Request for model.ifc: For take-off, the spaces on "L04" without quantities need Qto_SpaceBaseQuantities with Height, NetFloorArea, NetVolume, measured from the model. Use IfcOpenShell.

First a look at what the model holds.

```python
import ifcopenshell
import ifcopenshell.util.element
import ifcopenshell.util.unit

model = ifcopenshell.open("model.ifc")
print(model.schema)
for unit_type in ("LENGTHUNIT", "AREAUNIT", "VOLUMEUNIT"):
    print(unit_type, ifcopenshell.util.unit.calculate_unit_scale(model, unit_type))
storey = next(s for s in model.by_type("IfcBuildingStorey") if s.Name == "L04")
spaces = [e for e in ifcopenshell.util.element.get_decomposition(storey) if e.is_a("IfcSpace")]
for e in sorted(spaces, key=lambda e: e.id()):
    print(e.id(), e.is_a(), e.Name, list(ifcopenshell.util.element.get_psets(e, qtos_only=True)), sep=" | ")
```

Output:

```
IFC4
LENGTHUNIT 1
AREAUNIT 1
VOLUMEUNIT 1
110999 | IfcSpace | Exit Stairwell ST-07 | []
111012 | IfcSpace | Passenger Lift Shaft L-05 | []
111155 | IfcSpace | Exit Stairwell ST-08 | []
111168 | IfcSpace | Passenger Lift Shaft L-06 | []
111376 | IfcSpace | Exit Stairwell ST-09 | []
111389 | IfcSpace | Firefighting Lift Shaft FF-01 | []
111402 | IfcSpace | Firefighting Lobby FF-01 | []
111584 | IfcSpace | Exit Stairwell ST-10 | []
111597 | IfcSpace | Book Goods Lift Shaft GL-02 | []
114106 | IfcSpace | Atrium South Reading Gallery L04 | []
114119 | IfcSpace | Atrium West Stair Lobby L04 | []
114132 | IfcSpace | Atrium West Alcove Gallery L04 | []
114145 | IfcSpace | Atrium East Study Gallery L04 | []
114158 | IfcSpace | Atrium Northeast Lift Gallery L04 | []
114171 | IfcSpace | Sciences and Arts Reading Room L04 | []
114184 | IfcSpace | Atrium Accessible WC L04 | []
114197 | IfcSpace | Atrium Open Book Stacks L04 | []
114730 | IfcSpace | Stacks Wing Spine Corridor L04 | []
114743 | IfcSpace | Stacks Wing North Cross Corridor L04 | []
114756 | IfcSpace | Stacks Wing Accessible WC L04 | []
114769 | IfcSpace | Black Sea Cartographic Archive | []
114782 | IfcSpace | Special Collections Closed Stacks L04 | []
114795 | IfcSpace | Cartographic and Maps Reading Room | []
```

```python
import ifcopenshell
import ifcopenshell.api.pset
import ifcopenshell.geom
import ifcopenshell.util.element
import ifcopenshell.util.shape
import ifcopenshell.util.unit

model = ifcopenshell.open("model.ifc")
unit_scale = ifcopenshell.util.unit.calculate_unit_scale(model)
area_scale = ifcopenshell.util.unit.calculate_unit_scale(model, "AREAUNIT")
volume_scale = ifcopenshell.util.unit.calculate_unit_scale(model, "VOLUMEUNIT")
settings = ifcopenshell.geom.settings()

storey = next(s for s in model.by_type("IfcBuildingStorey") if s.Name == "L04")
spaces = [e for e in ifcopenshell.util.element.get_decomposition(storey) if e.is_a("IfcSpace")]

for e in sorted(spaces, key=lambda e: e.id()):
    if ifcopenshell.util.element.get_psets(e, qtos_only=True, should_inherit=False):
        continue
    # Geometry comes back in metres, in the element's own axes.
    shape = ifcopenshell.geom.create_shape(settings, e)
    values = {
        "Height": ifcopenshell.util.shape.get_z(shape.geometry) / unit_scale,
        "NetFloorArea": ifcopenshell.util.shape.get_footprint_area(shape.geometry) / area_scale,
        "NetVolume": ifcopenshell.util.shape.get_volume(shape.geometry) / volume_scale,
    }
    qto = ifcopenshell.api.pset.add_qto(model, product=e, name="Qto_SpaceBaseQuantities")
    ifcopenshell.api.pset.edit_qto(model, qto=qto, properties=values)
    print(e.id(), {k: round(v, 3) for k, v in values.items()})

model.write("model-out.ifc")
```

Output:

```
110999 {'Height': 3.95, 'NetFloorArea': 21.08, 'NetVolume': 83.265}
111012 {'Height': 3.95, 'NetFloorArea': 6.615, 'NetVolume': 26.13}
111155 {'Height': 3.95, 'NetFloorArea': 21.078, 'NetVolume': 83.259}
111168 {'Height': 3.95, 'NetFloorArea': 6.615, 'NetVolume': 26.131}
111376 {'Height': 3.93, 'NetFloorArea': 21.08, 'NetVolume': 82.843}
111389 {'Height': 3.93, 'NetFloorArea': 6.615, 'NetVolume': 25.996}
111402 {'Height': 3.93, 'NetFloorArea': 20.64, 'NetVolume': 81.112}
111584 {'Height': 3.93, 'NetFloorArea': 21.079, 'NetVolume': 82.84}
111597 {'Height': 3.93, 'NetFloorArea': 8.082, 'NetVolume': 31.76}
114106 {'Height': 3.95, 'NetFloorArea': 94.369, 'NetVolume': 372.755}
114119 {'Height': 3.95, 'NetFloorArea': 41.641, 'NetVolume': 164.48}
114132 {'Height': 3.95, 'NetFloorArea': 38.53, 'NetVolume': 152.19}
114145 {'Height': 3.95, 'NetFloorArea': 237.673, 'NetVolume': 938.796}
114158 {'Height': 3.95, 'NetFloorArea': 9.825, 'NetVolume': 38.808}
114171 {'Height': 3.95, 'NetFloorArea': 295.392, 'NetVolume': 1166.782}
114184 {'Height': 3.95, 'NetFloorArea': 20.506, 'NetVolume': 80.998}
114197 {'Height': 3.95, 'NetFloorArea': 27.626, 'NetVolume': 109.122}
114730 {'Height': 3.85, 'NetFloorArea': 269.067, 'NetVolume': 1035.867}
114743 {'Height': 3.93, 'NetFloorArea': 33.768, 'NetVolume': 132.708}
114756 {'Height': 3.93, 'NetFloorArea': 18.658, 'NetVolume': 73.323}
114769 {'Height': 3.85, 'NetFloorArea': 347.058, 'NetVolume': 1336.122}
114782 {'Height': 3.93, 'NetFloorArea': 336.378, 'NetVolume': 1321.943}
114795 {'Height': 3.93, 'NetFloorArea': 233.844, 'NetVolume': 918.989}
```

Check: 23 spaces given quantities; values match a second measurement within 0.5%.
